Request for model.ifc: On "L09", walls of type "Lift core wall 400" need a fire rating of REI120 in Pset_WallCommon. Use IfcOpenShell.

First a look at what the model holds.

```python
import ifcopenshell
import ifcopenshell.util.element

model = ifcopenshell.open("model.ifc")
print(model.schema)
storey = next(s for s in model.by_type("IfcBuildingStorey") if s.Name == "L09")
walls = [e for e in ifcopenshell.util.element.get_decomposition(storey) if e.is_a("IfcWall")]
seen = {}
for e in walls:
    element_type = ifcopenshell.util.element.get_type(e)
    key = (element_type.Name if element_type != e and element_type else None, ifcopenshell.util.element.get_pset(e, "Pset_WallCommon", "FireRating"))
    seen[key] = seen.get(key, 0) + 1
for (name, value), count in sorted(seen.items(), key=str):
    print(count, "x", name, "|", value)
```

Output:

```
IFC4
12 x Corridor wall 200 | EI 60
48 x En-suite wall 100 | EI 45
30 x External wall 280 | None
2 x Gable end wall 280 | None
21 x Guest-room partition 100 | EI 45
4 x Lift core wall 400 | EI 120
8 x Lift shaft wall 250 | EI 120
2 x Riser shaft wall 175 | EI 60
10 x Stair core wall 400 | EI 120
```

```python
import ifcopenshell
import ifcopenshell.api.pset
import ifcopenshell.util.element

model = ifcopenshell.open("model.ifc")

storey = next(s for s in model.by_type("IfcBuildingStorey") if s.Name == "L09")
walls = [e for e in ifcopenshell.util.element.get_decomposition(storey) if e.is_a("IfcWall")]

count = 0
for e in walls:
    element_type = ifcopenshell.util.element.get_type(e)
    if element_type in (None, e) or element_type.Name != "Lift core wall 400":
        continue
    # add_pset returns the element's existing set when there is one.
    pset = ifcopenshell.api.pset.add_pset(model, product=e, name="Pset_WallCommon")
    ifcopenshell.api.pset.edit_pset(model, pset=pset, properties={"FireRating": "REI120"})
    count += 1

print(count, "walls updated")

model.write("model_edited.ifc")
```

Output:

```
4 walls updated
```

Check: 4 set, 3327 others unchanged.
